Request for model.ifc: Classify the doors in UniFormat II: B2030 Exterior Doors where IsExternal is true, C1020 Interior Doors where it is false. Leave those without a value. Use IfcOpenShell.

First a look at what the model holds.

```python
import ifcopenshell
import ifcopenshell.util.element

model = ifcopenshell.open("model.ifc")
print(model.schema)
print("classifications:", [c.Name for c in model.by_type("IfcClassification")])
values = [ifcopenshell.util.element.get_pset(e, "Pset_DoorCommon", "IsExternal") for e in model.by_type("IfcDoor")]
for value in (True, False, None):
    print("IsExternal", value, values.count(value))
```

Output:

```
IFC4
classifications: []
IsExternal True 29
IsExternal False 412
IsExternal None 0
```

```python
import ifcopenshell
import ifcopenshell.api.classification
import ifcopenshell.util.element

model = ifcopenshell.open("model.ifc")

system = ifcopenshell.api.classification.add_classification(model, classification="UniFormat II")

doors = model.by_type("IfcDoor")
external = {e: ifcopenshell.util.element.get_pset(e, "Pset_DoorCommon", "IsExternal") for e in doors}
for flag, code, name in ((True, "B2030", "Exterior Doors"), (False, "C1020", "Interior Doors")):
    products = [e for e in doors if external[e] is flag]
    ifcopenshell.api.classification.add_reference(
        model, products=products, classification=system, identification=code, name=name
    )
    print(code, len(products))

model.write("model_updated.ifc")
```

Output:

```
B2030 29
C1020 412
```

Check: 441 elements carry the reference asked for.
